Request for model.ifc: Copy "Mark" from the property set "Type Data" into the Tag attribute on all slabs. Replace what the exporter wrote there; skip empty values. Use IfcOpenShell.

First a look at what the model holds.

```python
import ifcopenshell
import ifcopenshell.util.element

model = ifcopenshell.open("model.ifc")
print(model.schema)
slabs = model.by_type("IfcSlab")
print(len(slabs), "slabs")
for e in slabs[:8]:
    source = ifcopenshell.util.element.get_pset(e, "Type Data", "Mark")
    target = e.Tag
    print(e.id(), repr(source), repr(target), sep=" | ")
```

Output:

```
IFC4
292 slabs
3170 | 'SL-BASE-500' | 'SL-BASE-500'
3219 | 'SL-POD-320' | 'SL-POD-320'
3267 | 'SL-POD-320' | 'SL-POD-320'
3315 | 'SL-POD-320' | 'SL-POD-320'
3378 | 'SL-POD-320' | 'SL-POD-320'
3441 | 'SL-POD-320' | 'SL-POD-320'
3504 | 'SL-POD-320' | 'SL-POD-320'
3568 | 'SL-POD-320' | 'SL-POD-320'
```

```python
import ifcopenshell
import ifcopenshell.util.element

model = ifcopenshell.open("model.ifc")

count = 0
for e in model.by_type("IfcSlab"):
    value = ifcopenshell.util.element.get_pset(e, "Type Data", "Mark")
    current = e.Tag
    if not value or not value.strip() or current == value:
        continue
    e.Tag = value
    count += 1

print(count, "slabs updated")

model.write("model_rev.ifc")
```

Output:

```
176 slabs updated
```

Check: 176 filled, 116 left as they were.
